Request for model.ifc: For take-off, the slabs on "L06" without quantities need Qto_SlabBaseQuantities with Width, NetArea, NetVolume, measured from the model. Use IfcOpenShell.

First a look at what the model holds.

```python
import ifcopenshell
import ifcopenshell.util.element
import ifcopenshell.util.unit

model = ifcopenshell.open("model.ifc")
print(model.schema)
for unit_type in ("LENGTHUNIT", "AREAUNIT", "VOLUMEUNIT"):
    print(unit_type, ifcopenshell.util.unit.calculate_unit_scale(model, unit_type))
storey = next(s for s in model.by_type("IfcBuildingStorey") if s.Name == "L06")
slabs = [e for e in ifcopenshell.util.element.get_decomposition(storey) if e.is_a("IfcSlab")]
for e in sorted(slabs, key=lambda e: e.id()):
    print(e.id(), e.is_a(), e.Name, list(ifcopenshell.util.element.get_psets(e, qtos_only=True)), sep=" | ")
```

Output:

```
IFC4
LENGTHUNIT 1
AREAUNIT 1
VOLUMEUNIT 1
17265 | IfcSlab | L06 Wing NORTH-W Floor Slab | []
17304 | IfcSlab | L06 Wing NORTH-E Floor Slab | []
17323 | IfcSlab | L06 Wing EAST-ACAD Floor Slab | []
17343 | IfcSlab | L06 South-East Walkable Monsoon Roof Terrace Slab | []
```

```python
import ifcopenshell
import ifcopenshell.api.pset
import ifcopenshell.geom
import ifcopenshell.util.element
import ifcopenshell.util.shape
import ifcopenshell.util.unit

model = ifcopenshell.open("model.ifc")
unit_scale = ifcopenshell.util.unit.calculate_unit_scale(model)
area_scale = ifcopenshell.util.unit.calculate_unit_scale(model, "AREAUNIT")
volume_scale = ifcopenshell.util.unit.calculate_unit_scale(model, "VOLUMEUNIT")
settings = ifcopenshell.geom.settings()

storey = next(s for s in model.by_type("IfcBuildingStorey") if s.Name == "L06")
slabs = [e for e in ifcopenshell.util.element.get_decomposition(storey) if e.is_a("IfcSlab")]

for e in sorted(slabs, key=lambda e: e.id()):
    if ifcopenshell.util.element.get_psets(e, qtos_only=True, should_inherit=False):
        continue
    # Geometry comes back in metres, in the element's own axes.
    shape = ifcopenshell.geom.create_shape(settings, e)
    values = {
        "Width": ifcopenshell.util.shape.get_z(shape.geometry) / unit_scale,
        "NetArea": ifcopenshell.util.shape.get_footprint_area(shape.geometry) / area_scale,
        "NetVolume": ifcopenshell.util.shape.get_volume(shape.geometry) / volume_scale,
    }
    qto = ifcopenshell.api.pset.add_qto(model, product=e, name="Qto_SlabBaseQuantities")
    ifcopenshell.api.pset.edit_qto(model, qto=qto, properties=values)
    print(e.id(), {k: round(v, 3) for k, v in values.items()})

model.write("model_v2.ifc")
```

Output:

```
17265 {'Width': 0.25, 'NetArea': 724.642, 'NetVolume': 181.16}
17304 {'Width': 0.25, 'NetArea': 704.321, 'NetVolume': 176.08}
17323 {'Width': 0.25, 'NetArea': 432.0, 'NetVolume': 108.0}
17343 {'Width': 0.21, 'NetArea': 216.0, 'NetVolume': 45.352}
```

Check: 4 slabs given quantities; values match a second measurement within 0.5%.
